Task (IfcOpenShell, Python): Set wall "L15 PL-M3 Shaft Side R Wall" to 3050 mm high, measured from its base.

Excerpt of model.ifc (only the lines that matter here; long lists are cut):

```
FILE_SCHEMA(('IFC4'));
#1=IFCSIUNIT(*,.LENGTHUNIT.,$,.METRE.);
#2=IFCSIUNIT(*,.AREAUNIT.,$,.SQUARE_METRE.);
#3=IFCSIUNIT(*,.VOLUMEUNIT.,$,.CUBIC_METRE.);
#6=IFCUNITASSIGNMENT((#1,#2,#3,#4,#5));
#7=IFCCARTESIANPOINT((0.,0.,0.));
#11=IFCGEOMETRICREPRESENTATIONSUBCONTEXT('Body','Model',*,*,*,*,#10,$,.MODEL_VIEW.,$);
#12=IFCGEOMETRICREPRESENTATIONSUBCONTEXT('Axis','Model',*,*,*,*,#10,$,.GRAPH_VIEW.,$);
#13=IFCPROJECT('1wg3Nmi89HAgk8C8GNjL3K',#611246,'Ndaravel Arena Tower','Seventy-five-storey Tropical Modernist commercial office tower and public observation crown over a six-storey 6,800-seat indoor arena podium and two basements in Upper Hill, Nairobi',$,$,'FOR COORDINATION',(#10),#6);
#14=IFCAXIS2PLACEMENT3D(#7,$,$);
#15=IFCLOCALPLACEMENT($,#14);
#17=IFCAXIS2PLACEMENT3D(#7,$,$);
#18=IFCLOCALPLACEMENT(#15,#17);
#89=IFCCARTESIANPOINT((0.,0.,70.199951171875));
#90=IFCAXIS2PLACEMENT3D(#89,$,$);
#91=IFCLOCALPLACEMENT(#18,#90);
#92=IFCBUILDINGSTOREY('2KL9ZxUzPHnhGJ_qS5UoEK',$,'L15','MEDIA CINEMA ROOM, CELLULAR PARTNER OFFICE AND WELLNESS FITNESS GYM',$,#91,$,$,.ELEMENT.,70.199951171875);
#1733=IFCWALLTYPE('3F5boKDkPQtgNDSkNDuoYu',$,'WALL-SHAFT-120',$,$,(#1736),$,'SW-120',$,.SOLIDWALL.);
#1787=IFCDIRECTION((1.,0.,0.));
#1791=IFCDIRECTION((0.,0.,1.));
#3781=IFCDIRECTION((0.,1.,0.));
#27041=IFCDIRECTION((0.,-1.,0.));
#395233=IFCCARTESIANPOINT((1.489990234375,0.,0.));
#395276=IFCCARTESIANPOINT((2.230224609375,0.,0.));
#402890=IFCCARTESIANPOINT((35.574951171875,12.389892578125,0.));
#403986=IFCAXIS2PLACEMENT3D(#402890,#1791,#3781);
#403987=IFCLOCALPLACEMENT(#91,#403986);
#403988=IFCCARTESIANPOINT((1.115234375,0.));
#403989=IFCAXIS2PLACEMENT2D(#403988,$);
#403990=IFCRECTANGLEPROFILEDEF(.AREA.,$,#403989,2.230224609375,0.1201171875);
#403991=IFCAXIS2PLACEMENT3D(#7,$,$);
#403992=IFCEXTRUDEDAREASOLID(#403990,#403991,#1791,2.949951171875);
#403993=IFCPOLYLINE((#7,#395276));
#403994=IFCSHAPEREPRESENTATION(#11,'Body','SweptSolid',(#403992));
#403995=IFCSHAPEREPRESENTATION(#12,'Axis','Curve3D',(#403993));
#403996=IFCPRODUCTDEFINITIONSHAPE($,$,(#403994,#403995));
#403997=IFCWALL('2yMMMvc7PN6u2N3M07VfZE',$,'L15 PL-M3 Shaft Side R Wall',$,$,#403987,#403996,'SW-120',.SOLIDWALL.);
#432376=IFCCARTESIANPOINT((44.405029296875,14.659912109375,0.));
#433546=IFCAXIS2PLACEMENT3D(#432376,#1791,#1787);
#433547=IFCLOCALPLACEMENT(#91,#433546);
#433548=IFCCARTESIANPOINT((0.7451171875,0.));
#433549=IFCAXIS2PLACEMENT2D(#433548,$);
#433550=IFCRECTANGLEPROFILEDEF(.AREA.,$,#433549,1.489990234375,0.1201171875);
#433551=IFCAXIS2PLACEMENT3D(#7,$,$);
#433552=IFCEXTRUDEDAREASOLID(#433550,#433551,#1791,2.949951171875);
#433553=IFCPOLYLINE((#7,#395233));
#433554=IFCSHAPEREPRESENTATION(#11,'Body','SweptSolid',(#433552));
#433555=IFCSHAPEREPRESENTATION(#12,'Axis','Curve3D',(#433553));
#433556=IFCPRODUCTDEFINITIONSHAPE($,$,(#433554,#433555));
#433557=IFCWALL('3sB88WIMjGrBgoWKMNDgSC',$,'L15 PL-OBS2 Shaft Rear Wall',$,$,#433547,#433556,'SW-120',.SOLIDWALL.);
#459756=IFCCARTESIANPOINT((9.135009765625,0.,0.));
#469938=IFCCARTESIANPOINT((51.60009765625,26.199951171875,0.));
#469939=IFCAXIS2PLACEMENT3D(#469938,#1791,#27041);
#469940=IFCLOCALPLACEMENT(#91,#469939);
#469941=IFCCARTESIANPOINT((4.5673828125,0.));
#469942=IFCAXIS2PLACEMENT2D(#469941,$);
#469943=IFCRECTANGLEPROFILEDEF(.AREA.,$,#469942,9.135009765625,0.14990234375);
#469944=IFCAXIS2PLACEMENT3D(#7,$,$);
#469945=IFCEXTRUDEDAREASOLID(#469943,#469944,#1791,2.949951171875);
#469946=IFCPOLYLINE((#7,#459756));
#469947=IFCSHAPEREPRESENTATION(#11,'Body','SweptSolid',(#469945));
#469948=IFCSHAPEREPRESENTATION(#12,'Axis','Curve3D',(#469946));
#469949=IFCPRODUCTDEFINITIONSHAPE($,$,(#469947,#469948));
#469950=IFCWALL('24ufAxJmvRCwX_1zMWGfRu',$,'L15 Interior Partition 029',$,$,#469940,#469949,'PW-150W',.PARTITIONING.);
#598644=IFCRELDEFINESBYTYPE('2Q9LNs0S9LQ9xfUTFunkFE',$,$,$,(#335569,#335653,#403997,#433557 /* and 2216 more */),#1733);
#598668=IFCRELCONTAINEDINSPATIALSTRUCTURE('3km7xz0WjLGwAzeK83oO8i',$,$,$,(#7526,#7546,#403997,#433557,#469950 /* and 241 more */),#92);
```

```python
import ifcopenshell
import ifcopenshell.geom
import ifcopenshell.util.representation
import ifcopenshell.util.shape
import ifcopenshell.util.unit

model = ifcopenshell.open("model.ifc")
unit_scale = ifcopenshell.util.unit.calculate_unit_scale(model)
settings = ifcopenshell.geom.settings()


def volume(element):
    """Net volume in cubic metres, openings subtracted."""
    shape = ifcopenshell.geom.create_shape(settings, element)
    return ifcopenshell.util.shape.get_volume(shape.geometry)


wall = model.by_guid("2yMMMvc7PN6u2N3M07VfZE")
before = volume(wall)

body = ifcopenshell.util.representation.get_representation(wall, "Model", "Body")
solid = body.Items[0]
old_height = solid.Depth
solid.Depth = 3.05 / unit_scale
after = volume(wall)

print(f"height {old_height:g} -> {solid.Depth:g}, volume {before:.3f} -> {after:.3f} m3")

model.write("model_v2.ifc")
```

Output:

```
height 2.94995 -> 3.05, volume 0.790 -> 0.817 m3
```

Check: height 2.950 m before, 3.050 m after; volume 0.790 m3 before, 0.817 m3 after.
